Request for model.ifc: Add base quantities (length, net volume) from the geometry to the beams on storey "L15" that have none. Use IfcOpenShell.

First a look at what the model holds.

```python
import ifcopenshell
import ifcopenshell.util.element
import ifcopenshell.util.unit

model = ifcopenshell.open("model.ifc")
print(model.schema)
for unit_type in ("LENGTHUNIT", "AREAUNIT", "VOLUMEUNIT"):
    print(unit_type, ifcopenshell.util.unit.calculate_unit_scale(model, unit_type))
storey = next(s for s in model.by_type("IfcBuildingStorey") if s.Name == "L15")
beams = [e for e in ifcopenshell.util.element.get_decomposition(storey) if e.is_a("IfcBeam")]
for e in sorted(beams, key=lambda e: e.id()):
    print(e.id(), e.is_a(), e.Name, list(ifcopenshell.util.element.get_psets(e, qtos_only=True)), sep=" | ")
```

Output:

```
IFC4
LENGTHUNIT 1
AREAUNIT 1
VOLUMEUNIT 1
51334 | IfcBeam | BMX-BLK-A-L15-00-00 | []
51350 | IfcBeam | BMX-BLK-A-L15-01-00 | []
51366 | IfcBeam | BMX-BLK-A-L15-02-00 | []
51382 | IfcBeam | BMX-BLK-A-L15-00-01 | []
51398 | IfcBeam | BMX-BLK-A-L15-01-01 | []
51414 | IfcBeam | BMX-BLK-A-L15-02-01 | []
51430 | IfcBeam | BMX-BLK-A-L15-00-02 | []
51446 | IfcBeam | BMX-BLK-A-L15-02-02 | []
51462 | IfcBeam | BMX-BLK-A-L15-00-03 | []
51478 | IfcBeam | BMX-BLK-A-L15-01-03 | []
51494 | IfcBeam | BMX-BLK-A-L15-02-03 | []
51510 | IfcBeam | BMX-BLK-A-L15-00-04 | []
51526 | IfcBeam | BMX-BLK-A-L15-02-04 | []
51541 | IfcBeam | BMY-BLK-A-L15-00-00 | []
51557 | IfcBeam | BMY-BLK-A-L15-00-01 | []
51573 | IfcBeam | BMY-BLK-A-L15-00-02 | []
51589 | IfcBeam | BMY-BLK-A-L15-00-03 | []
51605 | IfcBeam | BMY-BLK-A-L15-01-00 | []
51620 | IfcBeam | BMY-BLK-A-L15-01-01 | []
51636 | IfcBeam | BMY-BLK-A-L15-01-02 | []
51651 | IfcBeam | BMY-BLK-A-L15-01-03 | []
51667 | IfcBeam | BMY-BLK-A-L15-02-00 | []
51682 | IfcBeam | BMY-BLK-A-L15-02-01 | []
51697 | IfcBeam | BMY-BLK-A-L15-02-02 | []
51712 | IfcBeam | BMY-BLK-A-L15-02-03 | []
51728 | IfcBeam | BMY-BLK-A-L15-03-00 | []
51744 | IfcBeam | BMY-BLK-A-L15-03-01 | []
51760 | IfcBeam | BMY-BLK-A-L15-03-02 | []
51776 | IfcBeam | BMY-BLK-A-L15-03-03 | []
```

```python
import ifcopenshell
import ifcopenshell.api.pset
import ifcopenshell.geom
import ifcopenshell.util.element
import ifcopenshell.util.shape
import ifcopenshell.util.unit

model = ifcopenshell.open("model.ifc")
unit_scale = ifcopenshell.util.unit.calculate_unit_scale(model)
volume_scale = ifcopenshell.util.unit.calculate_unit_scale(model, "VOLUMEUNIT")
settings = ifcopenshell.geom.settings()

storey = next(s for s in model.by_type("IfcBuildingStorey") if s.Name == "L15")
beams = [e for e in ifcopenshell.util.element.get_decomposition(storey) if e.is_a("IfcBeam")]

for e in sorted(beams, key=lambda e: e.id()):
    if ifcopenshell.util.element.get_psets(e, qtos_only=True, should_inherit=False):
        continue
    # Geometry comes back in metres, in the element's own axes.
    shape = ifcopenshell.geom.create_shape(settings, e)
    values = {
        "Length": ifcopenshell.util.shape.get_max_xyz(shape.geometry) / unit_scale,
        "NetVolume": ifcopenshell.util.shape.get_volume(shape.geometry) / volume_scale,
    }
    qto = ifcopenshell.api.pset.add_qto(model, product=e, name="Qto_BeamBaseQuantities")
    ifcopenshell.api.pset.edit_qto(model, qto=qto, properties=values)
    print(e.id(), {k: round(v, 3) for k, v in values.items()})

model.write("model_updated.ifc")
```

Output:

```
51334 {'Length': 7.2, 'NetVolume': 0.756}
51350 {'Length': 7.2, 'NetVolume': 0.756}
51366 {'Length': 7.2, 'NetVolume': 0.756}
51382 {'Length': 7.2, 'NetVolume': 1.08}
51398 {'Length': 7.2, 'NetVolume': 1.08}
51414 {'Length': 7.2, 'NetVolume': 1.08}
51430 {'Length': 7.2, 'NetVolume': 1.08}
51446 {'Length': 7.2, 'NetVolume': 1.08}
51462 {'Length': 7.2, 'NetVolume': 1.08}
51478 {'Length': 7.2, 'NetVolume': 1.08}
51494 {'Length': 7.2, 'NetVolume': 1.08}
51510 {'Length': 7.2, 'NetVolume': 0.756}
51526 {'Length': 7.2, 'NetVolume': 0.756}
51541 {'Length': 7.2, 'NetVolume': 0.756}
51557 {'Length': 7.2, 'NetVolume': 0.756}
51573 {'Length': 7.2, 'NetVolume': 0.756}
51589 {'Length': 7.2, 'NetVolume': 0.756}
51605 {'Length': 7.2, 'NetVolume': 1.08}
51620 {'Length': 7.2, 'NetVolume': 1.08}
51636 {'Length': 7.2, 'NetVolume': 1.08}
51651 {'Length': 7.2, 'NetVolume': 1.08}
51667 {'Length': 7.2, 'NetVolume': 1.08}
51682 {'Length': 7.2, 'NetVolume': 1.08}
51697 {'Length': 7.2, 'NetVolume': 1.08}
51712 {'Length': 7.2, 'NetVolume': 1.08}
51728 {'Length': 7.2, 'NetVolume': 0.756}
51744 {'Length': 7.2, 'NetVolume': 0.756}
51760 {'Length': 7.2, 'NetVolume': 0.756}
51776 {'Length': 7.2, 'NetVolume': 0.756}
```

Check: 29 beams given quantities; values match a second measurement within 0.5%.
